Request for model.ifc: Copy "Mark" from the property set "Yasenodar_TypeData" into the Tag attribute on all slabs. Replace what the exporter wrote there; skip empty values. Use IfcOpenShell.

First a look at what the model holds.

```python
import ifcopenshell
import ifcopenshell.util.element

model = ifcopenshell.open("model.ifc")
print(model.schema)
slabs = model.by_type("IfcSlab")
print(len(slabs), "slabs")
for e in slabs[:8]:
    source = ifcopenshell.util.element.get_pset(e, "Yasenodar_TypeData", "Mark")
    target = e.Tag
    print(e.id(), repr(source), repr(target), sep=" | ")
```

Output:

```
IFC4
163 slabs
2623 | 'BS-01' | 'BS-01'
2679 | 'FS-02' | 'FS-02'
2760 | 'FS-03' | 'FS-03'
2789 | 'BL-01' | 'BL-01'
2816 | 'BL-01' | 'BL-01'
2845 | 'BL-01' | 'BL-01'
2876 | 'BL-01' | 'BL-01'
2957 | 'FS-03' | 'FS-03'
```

```python
import ifcopenshell
import ifcopenshell.util.element

model = ifcopenshell.open("model.ifc")

count = 0
for e in model.by_type("IfcSlab"):
    value = ifcopenshell.util.element.get_pset(e, "Yasenodar_TypeData", "Mark")
    current = e.Tag
    if not value or not value.strip() or current == value:
        continue
    e.Tag = value
    count += 1

print(count, "slabs updated")

model.write("model_rev.ifc")
```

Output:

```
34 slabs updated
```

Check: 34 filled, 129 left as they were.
